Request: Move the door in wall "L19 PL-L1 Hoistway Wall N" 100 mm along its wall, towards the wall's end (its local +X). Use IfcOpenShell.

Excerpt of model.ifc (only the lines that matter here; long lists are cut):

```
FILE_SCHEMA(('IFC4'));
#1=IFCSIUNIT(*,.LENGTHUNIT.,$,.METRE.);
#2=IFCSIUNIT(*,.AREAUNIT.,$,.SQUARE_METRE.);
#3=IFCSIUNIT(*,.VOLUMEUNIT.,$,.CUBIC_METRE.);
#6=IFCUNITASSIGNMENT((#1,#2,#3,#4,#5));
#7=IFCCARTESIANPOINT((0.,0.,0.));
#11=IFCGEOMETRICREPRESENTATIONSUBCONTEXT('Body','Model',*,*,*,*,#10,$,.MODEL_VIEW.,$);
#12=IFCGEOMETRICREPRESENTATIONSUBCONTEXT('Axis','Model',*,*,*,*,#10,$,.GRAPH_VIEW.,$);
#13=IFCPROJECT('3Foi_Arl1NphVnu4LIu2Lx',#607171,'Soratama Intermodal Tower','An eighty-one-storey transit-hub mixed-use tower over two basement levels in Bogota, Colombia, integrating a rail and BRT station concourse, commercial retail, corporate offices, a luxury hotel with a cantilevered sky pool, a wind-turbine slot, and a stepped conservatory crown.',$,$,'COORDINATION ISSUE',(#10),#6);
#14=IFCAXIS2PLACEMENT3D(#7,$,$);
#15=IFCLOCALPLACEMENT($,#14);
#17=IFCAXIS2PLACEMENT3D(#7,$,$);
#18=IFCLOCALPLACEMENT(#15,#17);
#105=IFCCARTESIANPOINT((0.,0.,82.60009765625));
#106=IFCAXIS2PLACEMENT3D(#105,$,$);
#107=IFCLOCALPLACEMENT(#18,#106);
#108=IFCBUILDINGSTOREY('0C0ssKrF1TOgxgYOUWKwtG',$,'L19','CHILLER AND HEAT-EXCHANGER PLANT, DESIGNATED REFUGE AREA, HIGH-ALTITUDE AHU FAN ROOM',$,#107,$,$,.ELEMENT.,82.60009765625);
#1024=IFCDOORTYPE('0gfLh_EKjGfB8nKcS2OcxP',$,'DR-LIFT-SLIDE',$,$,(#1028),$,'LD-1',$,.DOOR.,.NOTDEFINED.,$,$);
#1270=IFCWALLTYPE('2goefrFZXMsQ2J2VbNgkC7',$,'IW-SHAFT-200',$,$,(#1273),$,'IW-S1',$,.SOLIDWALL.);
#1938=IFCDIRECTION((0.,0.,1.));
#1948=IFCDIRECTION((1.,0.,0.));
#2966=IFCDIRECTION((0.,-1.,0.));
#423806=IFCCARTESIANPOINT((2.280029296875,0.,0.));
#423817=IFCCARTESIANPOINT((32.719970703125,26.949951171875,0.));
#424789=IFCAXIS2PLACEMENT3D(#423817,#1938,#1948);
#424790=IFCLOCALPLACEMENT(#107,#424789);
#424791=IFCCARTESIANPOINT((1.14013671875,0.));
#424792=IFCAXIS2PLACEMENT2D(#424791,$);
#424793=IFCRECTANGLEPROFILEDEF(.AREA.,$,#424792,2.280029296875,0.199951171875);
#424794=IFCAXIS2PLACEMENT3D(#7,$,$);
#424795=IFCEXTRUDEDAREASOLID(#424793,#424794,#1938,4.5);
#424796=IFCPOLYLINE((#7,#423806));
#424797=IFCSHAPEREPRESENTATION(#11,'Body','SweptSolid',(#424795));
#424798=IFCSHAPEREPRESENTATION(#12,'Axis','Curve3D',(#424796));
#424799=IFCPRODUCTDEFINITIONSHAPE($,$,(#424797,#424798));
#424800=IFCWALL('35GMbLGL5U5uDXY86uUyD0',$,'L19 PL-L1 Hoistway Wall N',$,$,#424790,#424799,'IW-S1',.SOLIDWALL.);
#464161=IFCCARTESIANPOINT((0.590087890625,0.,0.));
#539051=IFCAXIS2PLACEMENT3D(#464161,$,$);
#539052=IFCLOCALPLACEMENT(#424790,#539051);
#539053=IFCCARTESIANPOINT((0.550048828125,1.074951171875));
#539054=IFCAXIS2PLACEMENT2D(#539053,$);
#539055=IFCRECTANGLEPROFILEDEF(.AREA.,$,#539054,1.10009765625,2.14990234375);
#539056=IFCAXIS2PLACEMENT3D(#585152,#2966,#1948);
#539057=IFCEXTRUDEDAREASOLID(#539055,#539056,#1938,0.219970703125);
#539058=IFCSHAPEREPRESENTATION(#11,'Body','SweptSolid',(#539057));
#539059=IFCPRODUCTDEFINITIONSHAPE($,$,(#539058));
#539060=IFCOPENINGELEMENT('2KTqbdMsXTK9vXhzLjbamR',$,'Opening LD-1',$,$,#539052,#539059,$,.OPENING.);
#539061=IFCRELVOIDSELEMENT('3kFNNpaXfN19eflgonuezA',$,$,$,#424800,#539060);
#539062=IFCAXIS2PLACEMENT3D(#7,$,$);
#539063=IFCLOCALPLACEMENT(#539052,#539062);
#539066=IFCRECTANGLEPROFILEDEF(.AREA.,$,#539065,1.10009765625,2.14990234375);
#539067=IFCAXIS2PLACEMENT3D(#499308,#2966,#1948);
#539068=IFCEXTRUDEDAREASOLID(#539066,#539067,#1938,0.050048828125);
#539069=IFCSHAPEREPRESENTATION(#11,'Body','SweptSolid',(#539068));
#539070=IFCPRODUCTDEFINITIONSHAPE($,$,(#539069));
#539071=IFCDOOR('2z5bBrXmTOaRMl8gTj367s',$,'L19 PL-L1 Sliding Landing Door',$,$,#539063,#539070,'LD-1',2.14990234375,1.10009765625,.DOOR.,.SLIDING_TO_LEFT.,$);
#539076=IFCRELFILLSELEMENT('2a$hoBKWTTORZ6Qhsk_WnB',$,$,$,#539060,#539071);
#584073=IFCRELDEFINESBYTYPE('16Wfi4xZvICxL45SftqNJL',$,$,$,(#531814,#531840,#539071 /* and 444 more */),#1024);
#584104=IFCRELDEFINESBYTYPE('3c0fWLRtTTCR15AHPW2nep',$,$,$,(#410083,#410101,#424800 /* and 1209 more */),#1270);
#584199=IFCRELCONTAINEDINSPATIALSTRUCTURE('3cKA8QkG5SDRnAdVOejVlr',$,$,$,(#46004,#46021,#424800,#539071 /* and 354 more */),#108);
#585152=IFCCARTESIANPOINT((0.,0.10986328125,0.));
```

```python
import ifcopenshell
import ifcopenshell.api.geometry
import ifcopenshell.util.placement

model = ifcopenshell.open("model.ifc")

door = model.by_guid("2z5bBrXmTOaRMl8gTj367s")
opening = door.FillsVoids[0].RelatingOpeningElement
wall = opening.VoidsElements[0].RelatingBuildingElement

wall_matrix = ifcopenshell.util.placement.get_local_placement(wall.ObjectPlacement)
shift = wall_matrix[:3, 0] * 0.1
before = ifcopenshell.util.placement.get_local_placement(door.ObjectPlacement)[:3, 3].copy()

# The door is placed relative to its opening, so it follows when the opening moves.
matrix = ifcopenshell.util.placement.get_local_placement(opening.ObjectPlacement)
matrix[:3, 3] += shift
ifcopenshell.api.geometry.edit_object_placement(
    model, product=opening, matrix=matrix, is_si=False, should_transform_children=True
)

after = ifcopenshell.util.placement.get_local_placement(door.ObjectPlacement)[:3, 3]
print("door moved by", (after - before).round(3) + 0.0)

model.write("model_updated.ifc")
```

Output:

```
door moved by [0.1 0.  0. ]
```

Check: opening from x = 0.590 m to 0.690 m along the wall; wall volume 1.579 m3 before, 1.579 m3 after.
